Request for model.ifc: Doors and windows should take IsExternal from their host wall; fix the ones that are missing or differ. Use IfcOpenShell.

First a look at what the model holds.

```python
import ifcopenshell
import ifcopenshell.util.element

model = ifcopenshell.open("model.ifc")
print(model.schema)
seen = {}
for e in model.by_type("IfcDoor") + model.by_type("IfcWindow"):
    if not e.FillsVoids:
        continue
    host = e.FillsVoids[0].RelatingOpeningElement.VoidsElements[0].RelatingBuildingElement
    own = ifcopenshell.util.element.get_pset(e, f"Pset_{e.is_a()[3:].removesuffix('StandardCase')}Common", "IsExternal")
    wall = ifcopenshell.util.element.get_pset(host, "Pset_WallCommon", "IsExternal")
    seen[e.is_a(), own, wall] = seen.get((e.is_a(), own, wall), 0) + 1
for (cls, own, wall), count in sorted(seen.items(), key=str):
    print(count, cls, "IsExternal:", own, "| host wall:", wall)
```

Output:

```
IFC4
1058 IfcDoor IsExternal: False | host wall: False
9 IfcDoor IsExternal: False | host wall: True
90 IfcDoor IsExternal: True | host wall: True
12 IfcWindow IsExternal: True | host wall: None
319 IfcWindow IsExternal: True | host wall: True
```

```python
import ifcopenshell
import ifcopenshell.api.pset
import ifcopenshell.util.element

model = ifcopenshell.open("model.ifc")

count = 0
for ifc_class, pset_name in (("IfcDoor", "Pset_DoorCommon"), ("IfcWindow", "Pset_WindowCommon")):
    for e in model.by_type(ifc_class):
        if not e.FillsVoids:
            continue
        host = e.FillsVoids[0].RelatingOpeningElement.VoidsElements[0].RelatingBuildingElement
        external = ifcopenshell.util.element.get_pset(host, "Pset_WallCommon", "IsExternal")
        if external is None or ifcopenshell.util.element.get_pset(e, pset_name, "IsExternal") == external:
            continue
        pset = ifcopenshell.api.pset.add_pset(model, product=e, name=pset_name)
        ifcopenshell.api.pset.edit_pset(model, pset=pset, properties={"IsExternal": external})
        count += 1

print(count, "updated")

model.write("model-out.ifc")
```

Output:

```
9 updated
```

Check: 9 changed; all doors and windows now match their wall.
